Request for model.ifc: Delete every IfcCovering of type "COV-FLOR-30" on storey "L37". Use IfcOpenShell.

First a look at what the model holds.

```python
import ifcopenshell
import ifcopenshell.util.element

model = ifcopenshell.open("model.ifc")
print(model.schema)
storey = next(s for s in model.by_type("IfcBuildingStorey") if s.Name == "L37")
coverings = [e for e in ifcopenshell.util.element.get_decomposition(storey) if e.is_a("IfcCovering")]
seen = {}
for e in coverings:
    element_type = ifcopenshell.util.element.get_type(e)
    name = element_type.Name if element_type not in (None, e) else None
    seen[name] = seen.get(name, 0) + 1
for name, count in sorted(seen.items(), key=str):
    print(count, "x", name)
```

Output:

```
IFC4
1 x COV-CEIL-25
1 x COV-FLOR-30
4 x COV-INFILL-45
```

```python
import ifcopenshell
import ifcopenshell.api.root
import ifcopenshell.util.element

model = ifcopenshell.open("model.ifc")

storey = next(s for s in model.by_type("IfcBuildingStorey") if s.Name == "L37")
coverings = [e for e in ifcopenshell.util.element.get_decomposition(storey) if e.is_a("IfcCovering")]
targets = [e for e in coverings if (t := ifcopenshell.util.element.get_type(e)) not in (None, e) and t.Name == "COV-FLOR-30"]

for e in targets:
    ifcopenshell.api.root.remove_product(model, product=e)
print(len(targets), "removed")

model.write("model_v2.ifc")
```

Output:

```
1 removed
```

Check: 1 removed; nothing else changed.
